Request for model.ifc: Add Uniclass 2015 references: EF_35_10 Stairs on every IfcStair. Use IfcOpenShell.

First a look at what the model holds.

```python
import ifcopenshell

model = ifcopenshell.open("model.ifc")
print(model.schema)
print("classifications:", [c.Name for c in model.by_type("IfcClassification")])
for ifc_class in ("IfcDoor", "IfcRoof", "IfcStair", "IfcWall", "IfcWindow"):
    print(ifc_class, len(model.by_type(ifc_class)))
```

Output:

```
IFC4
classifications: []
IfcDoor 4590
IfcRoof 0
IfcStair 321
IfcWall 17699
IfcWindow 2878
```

```python
import ifcopenshell
import ifcopenshell.api.classification

model = ifcopenshell.open("model.ifc")

system = ifcopenshell.api.classification.add_classification(model, classification="Uniclass 2015")

codes = {
    "IfcStair": ("EF_35_10", "Stairs"),
}
for ifc_class, (code, name) in codes.items():
    products = model.by_type(ifc_class)
    ifcopenshell.api.classification.add_reference(
        model, products=products, classification=system, identification=code, name=name
    )
    print(code, len(products))

model.write("model_edited.ifc")
```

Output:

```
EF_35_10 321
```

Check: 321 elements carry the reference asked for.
